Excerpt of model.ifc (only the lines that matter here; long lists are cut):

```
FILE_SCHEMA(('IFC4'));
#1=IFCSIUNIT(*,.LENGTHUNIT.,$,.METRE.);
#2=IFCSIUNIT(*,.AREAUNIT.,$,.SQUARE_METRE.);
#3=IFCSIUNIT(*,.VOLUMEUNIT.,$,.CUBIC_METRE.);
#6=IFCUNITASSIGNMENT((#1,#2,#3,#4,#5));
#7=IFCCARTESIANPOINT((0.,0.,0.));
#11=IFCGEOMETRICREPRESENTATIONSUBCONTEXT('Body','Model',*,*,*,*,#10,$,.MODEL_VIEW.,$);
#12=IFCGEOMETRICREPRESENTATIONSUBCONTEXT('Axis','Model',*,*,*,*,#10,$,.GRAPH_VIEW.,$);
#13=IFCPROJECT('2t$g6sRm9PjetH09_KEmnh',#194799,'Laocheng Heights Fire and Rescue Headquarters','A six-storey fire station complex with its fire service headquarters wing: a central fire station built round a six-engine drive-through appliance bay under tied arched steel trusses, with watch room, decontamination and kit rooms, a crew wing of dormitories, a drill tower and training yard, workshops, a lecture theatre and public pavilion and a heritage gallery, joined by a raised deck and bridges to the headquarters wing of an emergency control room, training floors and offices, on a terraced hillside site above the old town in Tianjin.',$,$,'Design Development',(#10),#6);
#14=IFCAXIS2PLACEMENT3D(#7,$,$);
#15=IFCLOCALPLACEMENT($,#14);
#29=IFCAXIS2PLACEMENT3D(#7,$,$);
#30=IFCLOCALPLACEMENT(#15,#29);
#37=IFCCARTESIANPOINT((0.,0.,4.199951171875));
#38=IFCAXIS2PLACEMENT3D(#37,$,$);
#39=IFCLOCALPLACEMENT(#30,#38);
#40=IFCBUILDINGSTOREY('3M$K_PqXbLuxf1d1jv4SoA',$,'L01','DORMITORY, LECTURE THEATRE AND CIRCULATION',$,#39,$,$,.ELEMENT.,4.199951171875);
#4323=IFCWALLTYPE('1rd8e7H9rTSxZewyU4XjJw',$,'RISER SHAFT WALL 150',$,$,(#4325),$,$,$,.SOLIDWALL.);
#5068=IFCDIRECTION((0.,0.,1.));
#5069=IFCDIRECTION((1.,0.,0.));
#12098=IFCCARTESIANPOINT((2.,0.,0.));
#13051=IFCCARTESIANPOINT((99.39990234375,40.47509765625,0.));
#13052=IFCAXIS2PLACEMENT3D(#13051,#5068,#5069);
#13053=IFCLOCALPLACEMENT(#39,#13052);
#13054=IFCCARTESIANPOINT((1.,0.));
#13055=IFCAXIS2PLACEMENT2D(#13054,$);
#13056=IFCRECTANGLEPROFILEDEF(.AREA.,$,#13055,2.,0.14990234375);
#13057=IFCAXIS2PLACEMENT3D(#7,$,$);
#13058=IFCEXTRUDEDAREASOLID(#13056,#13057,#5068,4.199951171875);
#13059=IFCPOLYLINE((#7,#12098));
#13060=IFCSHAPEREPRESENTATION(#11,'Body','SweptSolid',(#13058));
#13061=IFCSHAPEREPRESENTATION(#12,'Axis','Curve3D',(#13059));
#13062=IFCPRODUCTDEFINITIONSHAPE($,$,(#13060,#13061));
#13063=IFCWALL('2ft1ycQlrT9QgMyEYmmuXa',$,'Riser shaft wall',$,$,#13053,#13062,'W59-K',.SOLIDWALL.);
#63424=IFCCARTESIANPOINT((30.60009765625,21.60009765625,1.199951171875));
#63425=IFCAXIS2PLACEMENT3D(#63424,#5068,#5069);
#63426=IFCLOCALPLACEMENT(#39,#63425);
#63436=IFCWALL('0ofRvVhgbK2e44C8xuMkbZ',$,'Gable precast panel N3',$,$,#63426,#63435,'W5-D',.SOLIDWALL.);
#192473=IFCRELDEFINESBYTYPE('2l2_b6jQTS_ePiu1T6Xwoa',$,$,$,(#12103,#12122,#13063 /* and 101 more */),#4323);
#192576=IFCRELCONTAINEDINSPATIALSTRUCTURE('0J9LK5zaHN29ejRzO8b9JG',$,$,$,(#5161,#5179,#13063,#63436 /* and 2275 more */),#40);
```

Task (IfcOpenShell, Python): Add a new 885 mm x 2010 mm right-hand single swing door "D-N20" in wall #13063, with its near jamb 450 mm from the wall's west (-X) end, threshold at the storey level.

```python
import numpy as np
import ifcopenshell
import ifcopenshell.api.feature
import ifcopenshell.api.geometry
import ifcopenshell.api.root
import ifcopenshell.api.spatial
import ifcopenshell.geom
import ifcopenshell.util.element
import ifcopenshell.util.placement
import ifcopenshell.util.representation
import ifcopenshell.util.shape
import ifcopenshell.util.unit

model = ifcopenshell.open("model.ifc")
unit_scale = ifcopenshell.util.unit.calculate_unit_scale(model)
settings = ifcopenshell.geom.settings()


def volume(element):
    """Net volume in cubic metres, openings subtracted."""
    shape = ifcopenshell.geom.create_shape(settings, element)
    return ifcopenshell.util.shape.get_volume(shape.geometry)


wall = model.by_guid("2ft1ycQlrT9QgMyEYmmuXa")
storey = ifcopenshell.util.element.get_container(wall, ifc_class="IfcBuildingStorey")
context = ifcopenshell.util.representation.get_context(model, "Model", "Body", "MODEL_VIEW")
before = volume(wall)

width, height, from_end, sill = 0.885, 2.01, 0.45, 0.0  # metres

# The wall runs along its own X axis, and the end named is its -X end.
wall_shape = ifcopenshell.geom.create_shape(settings, wall)
x, y, z = ifcopenshell.util.shape.get_vertices(wall_shape.geometry).T
start = x.min() + from_end
face, thickness = float(y.min()), float(y.max() - y.min())
wall_matrix = ifcopenshell.util.placement.get_local_placement(wall.ObjectPlacement)
level = ifcopenshell.util.placement.get_local_placement(storey.ObjectPlacement)[2, 3]


def in_wall(x, y):
    """Placement at x, y metres in the wall's axes, at sill height."""
    matrix = wall_matrix.copy()
    matrix[:, 3] = wall_matrix @ np.array([x / unit_scale, y / unit_scale, 0.0, 1.0])
    matrix[2, 3] = level + sill / unit_scale
    return matrix


# Opening: a box that overshoots both wall faces by 50 mm.
opening = ifcopenshell.api.root.create_entity(model, ifc_class="IfcOpeningElement", predefined_type="OPENING")
box = ifcopenshell.api.geometry.add_wall_representation(
    model, context=context, length=width, height=height, thickness=thickness + 0.1
)
ifcopenshell.api.geometry.assign_representation(model, product=opening, representation=box)
ifcopenshell.api.geometry.edit_object_placement(model, product=opening, matrix=in_wall(start, face - 0.05), is_si=False)
ifcopenshell.api.feature.add_feature(model, feature=opening, element=wall)

door = ifcopenshell.api.root.create_entity(model, ifc_class="IfcDoor", name="D-N20", predefined_type="DOOR")
door.OverallWidth, door.OverallHeight = width / unit_scale, height / unit_scale
door.OperationType = "SINGLE_SWING_RIGHT"
body = ifcopenshell.api.geometry.add_door_representation(
    model,
    context=context,
    overall_width=door.OverallWidth,
    overall_height=door.OverallHeight,
    operation_type="SINGLE_SWING_RIGHT",
    lining_properties={"LiningDepth": thickness / unit_scale, "ThresholdDepth": thickness / unit_scale},
)
ifcopenshell.api.geometry.assign_representation(model, product=door, representation=body)
ifcopenshell.api.spatial.assign_container(model, products=[door], relating_structure=storey)
ifcopenshell.api.feature.add_filling(model, opening=opening, element=door)

# The lining spans the wall, so the door starts at the wall face.
ifcopenshell.api.geometry.edit_object_placement(model, product=door, matrix=in_wall(start, face), is_si=False)

after = volume(wall)

print(f"wall volume {before:.3f} -> {after:.3f} m3")

model.write("model_rev.ifc")
```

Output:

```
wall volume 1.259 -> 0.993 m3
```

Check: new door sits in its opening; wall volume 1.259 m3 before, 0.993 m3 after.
